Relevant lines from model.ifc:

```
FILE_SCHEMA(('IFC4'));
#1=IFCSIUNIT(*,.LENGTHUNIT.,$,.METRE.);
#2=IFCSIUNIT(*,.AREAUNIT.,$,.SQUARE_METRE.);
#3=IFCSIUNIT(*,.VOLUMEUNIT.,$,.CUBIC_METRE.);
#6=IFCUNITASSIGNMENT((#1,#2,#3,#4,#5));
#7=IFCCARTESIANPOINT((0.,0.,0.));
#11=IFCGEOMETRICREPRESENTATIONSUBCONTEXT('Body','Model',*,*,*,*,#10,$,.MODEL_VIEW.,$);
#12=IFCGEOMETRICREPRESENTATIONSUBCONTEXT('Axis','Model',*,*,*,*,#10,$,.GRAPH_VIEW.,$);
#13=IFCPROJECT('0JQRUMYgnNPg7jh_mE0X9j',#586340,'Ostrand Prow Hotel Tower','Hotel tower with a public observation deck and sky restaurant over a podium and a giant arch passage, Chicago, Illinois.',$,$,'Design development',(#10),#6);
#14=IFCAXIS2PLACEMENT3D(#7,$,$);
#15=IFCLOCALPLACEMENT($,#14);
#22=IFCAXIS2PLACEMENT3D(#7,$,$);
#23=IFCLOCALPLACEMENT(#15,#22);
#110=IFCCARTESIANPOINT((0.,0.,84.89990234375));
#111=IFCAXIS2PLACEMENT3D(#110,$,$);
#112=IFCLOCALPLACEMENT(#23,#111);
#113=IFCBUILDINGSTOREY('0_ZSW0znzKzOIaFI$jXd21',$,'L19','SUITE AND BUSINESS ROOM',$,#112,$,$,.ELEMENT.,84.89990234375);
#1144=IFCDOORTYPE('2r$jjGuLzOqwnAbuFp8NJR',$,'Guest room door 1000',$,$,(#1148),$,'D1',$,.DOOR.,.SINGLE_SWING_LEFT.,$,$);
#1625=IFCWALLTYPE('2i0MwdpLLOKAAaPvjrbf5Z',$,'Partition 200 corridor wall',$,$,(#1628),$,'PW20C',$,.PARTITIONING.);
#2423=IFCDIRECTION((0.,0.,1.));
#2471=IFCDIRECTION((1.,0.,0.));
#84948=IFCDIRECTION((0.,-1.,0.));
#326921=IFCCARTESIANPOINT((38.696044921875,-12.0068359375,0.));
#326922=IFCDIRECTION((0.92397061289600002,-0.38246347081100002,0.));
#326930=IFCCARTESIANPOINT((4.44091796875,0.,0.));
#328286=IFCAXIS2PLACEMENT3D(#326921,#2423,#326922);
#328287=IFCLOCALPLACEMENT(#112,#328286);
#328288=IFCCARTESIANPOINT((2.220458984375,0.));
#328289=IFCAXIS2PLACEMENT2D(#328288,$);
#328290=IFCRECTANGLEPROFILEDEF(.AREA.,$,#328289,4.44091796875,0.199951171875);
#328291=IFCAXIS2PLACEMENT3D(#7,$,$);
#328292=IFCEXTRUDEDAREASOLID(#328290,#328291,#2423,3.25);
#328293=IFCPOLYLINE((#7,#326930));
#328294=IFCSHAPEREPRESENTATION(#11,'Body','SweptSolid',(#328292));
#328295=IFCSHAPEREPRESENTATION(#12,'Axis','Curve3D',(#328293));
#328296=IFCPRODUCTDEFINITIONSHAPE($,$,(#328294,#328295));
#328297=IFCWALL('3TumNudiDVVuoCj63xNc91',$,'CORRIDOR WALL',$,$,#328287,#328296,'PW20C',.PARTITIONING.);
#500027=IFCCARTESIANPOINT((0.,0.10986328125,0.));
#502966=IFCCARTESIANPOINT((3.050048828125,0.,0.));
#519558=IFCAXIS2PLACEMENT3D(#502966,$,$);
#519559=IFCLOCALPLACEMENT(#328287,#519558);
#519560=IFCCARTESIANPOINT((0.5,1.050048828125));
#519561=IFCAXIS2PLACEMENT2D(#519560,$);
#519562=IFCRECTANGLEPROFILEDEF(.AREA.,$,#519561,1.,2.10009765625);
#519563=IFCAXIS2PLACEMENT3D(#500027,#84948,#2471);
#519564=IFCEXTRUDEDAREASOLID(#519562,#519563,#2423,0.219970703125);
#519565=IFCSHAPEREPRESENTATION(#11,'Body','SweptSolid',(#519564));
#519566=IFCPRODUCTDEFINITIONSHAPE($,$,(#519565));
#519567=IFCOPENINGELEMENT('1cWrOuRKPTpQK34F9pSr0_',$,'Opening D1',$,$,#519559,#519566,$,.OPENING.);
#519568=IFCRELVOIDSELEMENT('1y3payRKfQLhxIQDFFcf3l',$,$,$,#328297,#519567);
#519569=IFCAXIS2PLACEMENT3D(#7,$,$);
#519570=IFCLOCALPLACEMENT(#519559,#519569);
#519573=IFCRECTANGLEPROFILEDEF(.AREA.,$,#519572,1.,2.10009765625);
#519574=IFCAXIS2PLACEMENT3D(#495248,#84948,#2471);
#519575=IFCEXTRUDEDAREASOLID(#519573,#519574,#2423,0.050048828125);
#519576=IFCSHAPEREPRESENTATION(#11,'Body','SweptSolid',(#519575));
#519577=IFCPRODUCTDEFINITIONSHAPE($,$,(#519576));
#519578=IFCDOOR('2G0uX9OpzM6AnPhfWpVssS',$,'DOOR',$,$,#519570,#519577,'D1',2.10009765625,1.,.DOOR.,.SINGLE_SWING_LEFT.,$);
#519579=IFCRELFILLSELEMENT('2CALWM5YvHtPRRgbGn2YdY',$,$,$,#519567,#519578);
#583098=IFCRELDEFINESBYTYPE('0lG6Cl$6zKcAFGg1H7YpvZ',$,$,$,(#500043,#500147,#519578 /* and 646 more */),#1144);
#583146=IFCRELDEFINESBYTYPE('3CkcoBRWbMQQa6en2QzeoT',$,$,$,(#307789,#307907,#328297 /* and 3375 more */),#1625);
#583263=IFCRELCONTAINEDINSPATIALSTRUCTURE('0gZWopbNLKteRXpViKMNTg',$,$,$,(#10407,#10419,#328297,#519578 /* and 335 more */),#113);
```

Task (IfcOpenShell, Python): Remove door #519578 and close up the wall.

```python
import ifcopenshell
import ifcopenshell.api.feature
import ifcopenshell.api.root
import ifcopenshell.geom
import ifcopenshell.util.shape

model = ifcopenshell.open("model.ifc")
settings = ifcopenshell.geom.settings()


def volume(element):
    """Net volume in cubic metres, openings subtracted."""
    shape = ifcopenshell.geom.create_shape(settings, element)
    return ifcopenshell.util.shape.get_volume(shape.geometry)


door = model.by_guid("2G0uX9OpzM6AnPhfWpVssS")
opening = door.FillsVoids[0].RelatingOpeningElement
wall = opening.VoidsElements[0].RelatingBuildingElement
before = volume(wall)

ifcopenshell.api.root.remove_product(model, product=door)
ifcopenshell.api.feature.remove_feature(model, feature=opening)

after = volume(wall)

print(f"wall volume {before:.3f} -> {after:.3f} m3")

model.write("model_rev.ifc")
```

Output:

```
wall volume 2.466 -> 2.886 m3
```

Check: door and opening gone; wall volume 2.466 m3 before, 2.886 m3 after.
